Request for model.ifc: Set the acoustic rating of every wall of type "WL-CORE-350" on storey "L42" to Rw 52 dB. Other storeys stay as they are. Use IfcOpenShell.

First a look at what the model holds.

```python
import ifcopenshell
import ifcopenshell.util.element

model = ifcopenshell.open("model.ifc")
print(model.schema)
storey = next(s for s in model.by_type("IfcBuildingStorey") if s.Name == "L42")
walls = [e for e in ifcopenshell.util.element.get_decomposition(storey) if e.is_a("IfcWall")]
seen = {}
for e in walls:
    element_type = ifcopenshell.util.element.get_type(e)
    key = (element_type.Name if element_type != e and element_type else None, ifcopenshell.util.element.get_pset(e, "Pset_WallCommon", "AcousticRating"))
    seen[key] = seen.get(key, 0) + 1
for (name, value), count in sorted(seen.items(), key=str):
    print(count, "x", name, "|", value)
```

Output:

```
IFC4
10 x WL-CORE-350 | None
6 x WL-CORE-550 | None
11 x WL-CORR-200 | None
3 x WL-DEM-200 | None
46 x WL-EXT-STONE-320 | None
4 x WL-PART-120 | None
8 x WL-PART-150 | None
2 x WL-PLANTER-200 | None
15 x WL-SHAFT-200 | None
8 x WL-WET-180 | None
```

```python
import ifcopenshell
import ifcopenshell.api.pset
import ifcopenshell.util.element

model = ifcopenshell.open("model.ifc")

storey = next(s for s in model.by_type("IfcBuildingStorey") if s.Name == "L42")
walls = [e for e in ifcopenshell.util.element.get_decomposition(storey) if e.is_a("IfcWall")]

count = 0
for e in walls:
    element_type = ifcopenshell.util.element.get_type(e)
    if element_type in (None, e) or element_type.Name != "WL-CORE-350":
        continue
    # add_pset returns the element's existing set when there is one.
    pset = ifcopenshell.api.pset.add_pset(model, product=e, name="Pset_WallCommon")
    ifcopenshell.api.pset.edit_pset(model, pset=pset, properties={"AcousticRating": "Rw 52 dB"})
    count += 1

print(count, "walls updated")

model.write("model-out.ifc")
```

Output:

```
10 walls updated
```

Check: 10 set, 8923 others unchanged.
